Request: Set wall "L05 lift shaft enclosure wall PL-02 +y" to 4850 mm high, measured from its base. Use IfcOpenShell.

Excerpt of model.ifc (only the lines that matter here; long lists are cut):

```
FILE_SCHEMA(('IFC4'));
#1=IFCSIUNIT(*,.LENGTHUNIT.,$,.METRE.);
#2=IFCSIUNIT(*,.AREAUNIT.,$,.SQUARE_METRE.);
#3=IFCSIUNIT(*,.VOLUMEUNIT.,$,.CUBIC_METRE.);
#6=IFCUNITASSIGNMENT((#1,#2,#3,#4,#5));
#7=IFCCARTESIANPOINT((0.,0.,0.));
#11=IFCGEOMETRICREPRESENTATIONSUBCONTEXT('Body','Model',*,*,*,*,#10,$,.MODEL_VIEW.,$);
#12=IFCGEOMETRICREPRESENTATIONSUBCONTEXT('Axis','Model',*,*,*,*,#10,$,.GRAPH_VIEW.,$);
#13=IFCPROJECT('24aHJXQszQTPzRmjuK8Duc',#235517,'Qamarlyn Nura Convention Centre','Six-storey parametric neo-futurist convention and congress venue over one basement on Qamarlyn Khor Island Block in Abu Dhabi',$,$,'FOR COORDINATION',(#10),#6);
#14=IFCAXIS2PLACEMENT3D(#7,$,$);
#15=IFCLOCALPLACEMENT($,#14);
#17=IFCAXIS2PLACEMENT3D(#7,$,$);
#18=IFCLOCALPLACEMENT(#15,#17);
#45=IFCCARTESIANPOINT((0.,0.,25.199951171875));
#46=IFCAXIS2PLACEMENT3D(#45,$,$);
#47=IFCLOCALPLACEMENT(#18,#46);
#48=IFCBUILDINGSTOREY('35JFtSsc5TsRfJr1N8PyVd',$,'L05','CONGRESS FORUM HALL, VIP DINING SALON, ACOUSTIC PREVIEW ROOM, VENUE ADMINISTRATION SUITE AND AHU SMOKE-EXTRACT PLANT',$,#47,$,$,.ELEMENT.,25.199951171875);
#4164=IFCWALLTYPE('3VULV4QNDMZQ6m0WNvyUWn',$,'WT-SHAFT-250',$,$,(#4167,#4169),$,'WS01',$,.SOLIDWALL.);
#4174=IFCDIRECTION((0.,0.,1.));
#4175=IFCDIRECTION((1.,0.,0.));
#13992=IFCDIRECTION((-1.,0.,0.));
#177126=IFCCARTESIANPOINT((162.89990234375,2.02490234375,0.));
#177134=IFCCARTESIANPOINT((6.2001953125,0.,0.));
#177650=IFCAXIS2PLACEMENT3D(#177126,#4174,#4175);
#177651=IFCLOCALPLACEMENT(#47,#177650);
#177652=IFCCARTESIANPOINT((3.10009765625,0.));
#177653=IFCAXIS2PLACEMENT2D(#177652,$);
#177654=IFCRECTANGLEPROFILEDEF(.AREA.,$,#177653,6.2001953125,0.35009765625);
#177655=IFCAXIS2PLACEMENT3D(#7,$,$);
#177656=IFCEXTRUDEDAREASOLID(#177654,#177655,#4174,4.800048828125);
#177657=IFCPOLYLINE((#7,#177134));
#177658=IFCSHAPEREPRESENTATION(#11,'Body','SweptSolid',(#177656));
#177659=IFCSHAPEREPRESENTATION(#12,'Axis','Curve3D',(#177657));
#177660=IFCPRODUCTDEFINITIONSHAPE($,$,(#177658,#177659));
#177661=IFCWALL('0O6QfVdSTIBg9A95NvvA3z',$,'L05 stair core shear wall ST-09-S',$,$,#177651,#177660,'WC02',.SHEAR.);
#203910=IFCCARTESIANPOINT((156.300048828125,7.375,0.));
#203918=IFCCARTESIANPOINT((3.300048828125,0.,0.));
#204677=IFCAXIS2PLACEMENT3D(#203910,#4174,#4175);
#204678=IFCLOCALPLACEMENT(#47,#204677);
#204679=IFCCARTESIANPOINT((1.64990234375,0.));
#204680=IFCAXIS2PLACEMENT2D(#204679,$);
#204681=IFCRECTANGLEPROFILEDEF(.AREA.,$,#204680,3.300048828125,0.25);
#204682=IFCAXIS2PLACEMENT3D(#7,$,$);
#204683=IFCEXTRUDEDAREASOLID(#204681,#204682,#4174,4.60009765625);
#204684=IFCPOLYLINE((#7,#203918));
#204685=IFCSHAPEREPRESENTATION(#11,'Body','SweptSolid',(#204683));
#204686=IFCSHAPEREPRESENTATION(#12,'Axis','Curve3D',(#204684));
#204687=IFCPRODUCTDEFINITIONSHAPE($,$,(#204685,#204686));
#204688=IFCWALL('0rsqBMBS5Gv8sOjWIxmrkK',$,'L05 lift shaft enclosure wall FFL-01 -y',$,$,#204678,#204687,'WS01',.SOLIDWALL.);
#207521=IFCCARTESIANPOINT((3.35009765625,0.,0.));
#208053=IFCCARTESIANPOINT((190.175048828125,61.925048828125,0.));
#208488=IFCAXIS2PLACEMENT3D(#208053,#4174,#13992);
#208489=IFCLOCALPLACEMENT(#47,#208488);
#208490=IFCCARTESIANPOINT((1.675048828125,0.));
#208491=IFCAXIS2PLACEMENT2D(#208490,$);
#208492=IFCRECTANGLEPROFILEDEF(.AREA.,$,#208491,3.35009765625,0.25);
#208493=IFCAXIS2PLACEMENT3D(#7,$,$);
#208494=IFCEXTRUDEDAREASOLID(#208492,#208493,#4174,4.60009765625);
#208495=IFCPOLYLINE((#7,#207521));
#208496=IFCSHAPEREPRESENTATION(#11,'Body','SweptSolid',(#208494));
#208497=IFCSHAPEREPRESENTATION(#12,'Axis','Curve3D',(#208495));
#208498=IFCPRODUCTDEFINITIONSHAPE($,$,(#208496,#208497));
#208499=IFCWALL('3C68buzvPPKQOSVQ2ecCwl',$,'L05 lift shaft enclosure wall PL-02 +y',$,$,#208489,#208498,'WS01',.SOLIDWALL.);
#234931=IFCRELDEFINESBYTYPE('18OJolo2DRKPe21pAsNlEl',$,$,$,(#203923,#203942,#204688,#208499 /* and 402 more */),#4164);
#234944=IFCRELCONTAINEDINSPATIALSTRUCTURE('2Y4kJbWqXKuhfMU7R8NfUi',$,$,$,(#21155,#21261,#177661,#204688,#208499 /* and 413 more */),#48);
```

```python
import ifcopenshell
import ifcopenshell.geom
import ifcopenshell.util.representation
import ifcopenshell.util.shape

model = ifcopenshell.open("model.ifc")
settings = ifcopenshell.geom.settings()


def volume(element):
    """Net volume in cubic metres, openings subtracted."""
    shape = ifcopenshell.geom.create_shape(settings, element)
    return ifcopenshell.util.shape.get_volume(shape.geometry)


wall = model.by_guid("3C68buzvPPKQOSVQ2ecCwl")
before = volume(wall)

body = ifcopenshell.util.representation.get_representation(wall, "Model", "Body")
solid = body.Items[0]
old_height = solid.Depth
solid.Depth = 4.85
after = volume(wall)

print(f"height {old_height:g} -> {solid.Depth:g}, volume {before:.3f} -> {after:.3f} m3")

model.write("model_v2.ifc")
```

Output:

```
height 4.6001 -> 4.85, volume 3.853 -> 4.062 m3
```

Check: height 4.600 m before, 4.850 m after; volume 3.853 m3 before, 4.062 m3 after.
